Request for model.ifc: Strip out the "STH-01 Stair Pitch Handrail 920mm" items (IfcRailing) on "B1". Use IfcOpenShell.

First a look at what the model holds.

```python
import ifcopenshell
import ifcopenshell.util.element

model = ifcopenshell.open("model.ifc")
print(model.schema)
storey = next(s for s in model.by_type("IfcBuildingStorey") if s.Name == "B1")
railings = [e for e in ifcopenshell.util.element.get_decomposition(storey) if e.is_a("IfcRailing")]
seen = {}
for e in railings:
    element_type = ifcopenshell.util.element.get_type(e)
    name = element_type.Name if element_type not in (None, e) else None
    seen[name] = seen.get(name, 0) + 1
for name, count in sorted(seen.items(), key=str):
    print(count, "x", name)
```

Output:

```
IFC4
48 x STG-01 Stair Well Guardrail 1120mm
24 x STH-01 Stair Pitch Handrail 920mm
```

```python
import ifcopenshell
import ifcopenshell.api.root
import ifcopenshell.util.element

model = ifcopenshell.open("model.ifc")

storey = next(s for s in model.by_type("IfcBuildingStorey") if s.Name == "B1")
railings = [e for e in ifcopenshell.util.element.get_decomposition(storey) if e.is_a("IfcRailing")]
targets = [e for e in railings if (t := ifcopenshell.util.element.get_type(e)) not in (None, e) and t.Name == "STH-01 Stair Pitch Handrail 920mm"]

for e in targets:
    ifcopenshell.api.root.remove_product(model, product=e)
print(len(targets), "removed")

model.write("model-out.ifc")
```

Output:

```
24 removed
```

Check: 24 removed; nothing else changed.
